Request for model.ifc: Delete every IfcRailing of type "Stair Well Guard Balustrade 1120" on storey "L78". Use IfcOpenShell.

First a look at what the model holds.

```python
import ifcopenshell
import ifcopenshell.util.element

model = ifcopenshell.open("model.ifc")
print(model.schema)
storey = next(s for s in model.by_type("IfcBuildingStorey") if s.Name == "L78")
railings = [e for e in ifcopenshell.util.element.get_decomposition(storey) if e.is_a("IfcRailing")]
seen = {}
for e in railings:
    element_type = ifcopenshell.util.element.get_type(e)
    name = element_type.Name if element_type not in (None, e) else None
    seen[name] = seen.get(name, 0) + 1
for name, count in sorted(seen.items(), key=str):
    print(count, "x", name)
```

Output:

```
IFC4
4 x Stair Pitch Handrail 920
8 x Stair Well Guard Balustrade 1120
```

```python
import ifcopenshell
import ifcopenshell.api.root
import ifcopenshell.util.element

model = ifcopenshell.open("model.ifc")

storey = next(s for s in model.by_type("IfcBuildingStorey") if s.Name == "L78")
railings = [e for e in ifcopenshell.util.element.get_decomposition(storey) if e.is_a("IfcRailing")]
targets = [e for e in railings if (t := ifcopenshell.util.element.get_type(e)) not in (None, e) and t.Name == "Stair Well Guard Balustrade 1120"]

for e in targets:
    ifcopenshell.api.root.remove_product(model, product=e)
print(len(targets), "removed")

model.write("model-out.ifc")
```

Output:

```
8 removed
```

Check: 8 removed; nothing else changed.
